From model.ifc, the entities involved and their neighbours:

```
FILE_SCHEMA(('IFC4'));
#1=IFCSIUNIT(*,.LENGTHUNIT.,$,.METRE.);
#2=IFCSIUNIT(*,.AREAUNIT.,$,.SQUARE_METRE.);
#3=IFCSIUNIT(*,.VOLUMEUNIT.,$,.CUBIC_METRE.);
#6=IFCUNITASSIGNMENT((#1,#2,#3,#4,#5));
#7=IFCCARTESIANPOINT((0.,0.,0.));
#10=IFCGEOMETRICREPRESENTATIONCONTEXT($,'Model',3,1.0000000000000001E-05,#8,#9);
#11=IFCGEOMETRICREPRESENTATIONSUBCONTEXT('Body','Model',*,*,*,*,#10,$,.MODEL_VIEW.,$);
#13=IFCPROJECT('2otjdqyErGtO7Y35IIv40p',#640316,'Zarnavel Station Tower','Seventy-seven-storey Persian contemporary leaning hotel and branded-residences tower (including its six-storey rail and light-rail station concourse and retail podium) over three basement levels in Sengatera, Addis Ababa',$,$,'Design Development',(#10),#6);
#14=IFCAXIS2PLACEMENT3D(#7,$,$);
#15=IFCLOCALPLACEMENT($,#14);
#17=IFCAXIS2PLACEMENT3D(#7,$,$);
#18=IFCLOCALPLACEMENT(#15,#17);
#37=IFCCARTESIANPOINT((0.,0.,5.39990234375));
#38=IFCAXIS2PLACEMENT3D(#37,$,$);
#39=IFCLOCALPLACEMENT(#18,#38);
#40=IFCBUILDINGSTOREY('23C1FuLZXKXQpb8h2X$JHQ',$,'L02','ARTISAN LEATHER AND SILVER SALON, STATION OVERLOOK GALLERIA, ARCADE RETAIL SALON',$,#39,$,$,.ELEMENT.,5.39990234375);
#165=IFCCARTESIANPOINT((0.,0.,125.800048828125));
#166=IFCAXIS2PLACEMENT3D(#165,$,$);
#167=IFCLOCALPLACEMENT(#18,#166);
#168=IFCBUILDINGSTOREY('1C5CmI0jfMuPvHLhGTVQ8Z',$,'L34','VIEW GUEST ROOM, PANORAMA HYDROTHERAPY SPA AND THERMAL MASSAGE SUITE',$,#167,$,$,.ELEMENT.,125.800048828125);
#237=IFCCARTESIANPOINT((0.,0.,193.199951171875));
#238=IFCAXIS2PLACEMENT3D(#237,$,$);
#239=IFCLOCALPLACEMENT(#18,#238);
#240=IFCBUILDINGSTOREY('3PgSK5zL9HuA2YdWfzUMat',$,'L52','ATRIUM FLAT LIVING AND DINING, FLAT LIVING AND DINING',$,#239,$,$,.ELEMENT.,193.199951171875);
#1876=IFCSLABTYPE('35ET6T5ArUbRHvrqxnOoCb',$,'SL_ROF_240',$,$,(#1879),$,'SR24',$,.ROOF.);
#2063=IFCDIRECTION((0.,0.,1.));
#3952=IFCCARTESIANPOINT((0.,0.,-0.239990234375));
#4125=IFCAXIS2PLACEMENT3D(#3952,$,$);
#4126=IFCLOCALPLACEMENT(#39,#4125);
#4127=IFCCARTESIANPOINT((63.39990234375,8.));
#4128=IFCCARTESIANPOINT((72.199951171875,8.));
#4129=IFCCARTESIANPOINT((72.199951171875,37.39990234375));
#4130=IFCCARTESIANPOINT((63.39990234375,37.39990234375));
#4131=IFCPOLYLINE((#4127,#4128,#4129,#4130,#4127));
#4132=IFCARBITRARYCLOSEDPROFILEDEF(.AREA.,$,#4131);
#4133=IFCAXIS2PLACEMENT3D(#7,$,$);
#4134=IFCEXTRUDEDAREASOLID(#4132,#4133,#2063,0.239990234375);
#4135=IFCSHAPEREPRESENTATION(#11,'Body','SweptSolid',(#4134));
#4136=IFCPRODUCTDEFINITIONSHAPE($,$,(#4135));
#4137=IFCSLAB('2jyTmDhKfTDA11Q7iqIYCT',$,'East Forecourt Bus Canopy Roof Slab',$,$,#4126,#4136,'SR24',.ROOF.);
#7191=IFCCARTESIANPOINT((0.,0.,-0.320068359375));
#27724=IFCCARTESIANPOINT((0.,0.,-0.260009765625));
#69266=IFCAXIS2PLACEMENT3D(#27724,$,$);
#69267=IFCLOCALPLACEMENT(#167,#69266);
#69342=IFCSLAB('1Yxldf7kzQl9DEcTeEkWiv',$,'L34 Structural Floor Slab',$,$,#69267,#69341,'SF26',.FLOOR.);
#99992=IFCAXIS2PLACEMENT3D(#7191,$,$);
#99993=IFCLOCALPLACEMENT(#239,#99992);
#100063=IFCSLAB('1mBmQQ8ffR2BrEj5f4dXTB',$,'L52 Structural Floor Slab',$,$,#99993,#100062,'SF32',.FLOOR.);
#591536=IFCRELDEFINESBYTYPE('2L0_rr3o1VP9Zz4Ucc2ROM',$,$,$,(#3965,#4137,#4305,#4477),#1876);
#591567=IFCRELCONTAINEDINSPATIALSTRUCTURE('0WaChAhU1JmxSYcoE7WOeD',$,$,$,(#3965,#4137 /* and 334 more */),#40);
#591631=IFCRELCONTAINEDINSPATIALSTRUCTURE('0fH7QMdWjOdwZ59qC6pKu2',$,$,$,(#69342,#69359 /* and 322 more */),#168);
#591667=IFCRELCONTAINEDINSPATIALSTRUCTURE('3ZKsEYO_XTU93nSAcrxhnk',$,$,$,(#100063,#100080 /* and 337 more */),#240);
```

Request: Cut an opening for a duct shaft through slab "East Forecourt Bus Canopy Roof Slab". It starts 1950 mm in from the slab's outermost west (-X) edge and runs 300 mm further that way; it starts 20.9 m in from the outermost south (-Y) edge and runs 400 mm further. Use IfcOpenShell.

```python
import numpy as np
import ifcopenshell
import ifcopenshell.api.feature
import ifcopenshell.api.geometry
import ifcopenshell.api.root
import ifcopenshell.geom
import ifcopenshell.util.placement
import ifcopenshell.util.representation
import ifcopenshell.util.shape
import ifcopenshell.util.unit

model = ifcopenshell.open("model.ifc")
unit_scale = ifcopenshell.util.unit.calculate_unit_scale(model)
settings = ifcopenshell.geom.settings()


def volume(element):
    """Net volume in cubic metres, openings subtracted."""
    shape = ifcopenshell.geom.create_shape(settings, element)
    return ifcopenshell.util.shape.get_volume(shape.geometry)


slab = model.by_id(4137)
before = volume(slab)

# Extent in the slab's own axes, in metres. The edges named are its -X and -Y sides.
slab_shape = ifcopenshell.geom.create_shape(settings, slab)
vertices = ifcopenshell.util.shape.get_vertices(slab_shape.geometry)
x_min, y_min, bottom = vertices.min(axis=0)
top = vertices[:, 2].max()

opening = ifcopenshell.api.root.create_entity(model, ifc_class="IfcOpeningElement", name="Duct shaft opening", predefined_type="OPENING")
context = ifcopenshell.util.representation.get_context(model, "Model", "Body", "MODEL_VIEW")
width, depth = 0.3, 0.4
outline = [(0.0, 0.0), (width, 0.0), (width, depth), (0.0, depth), (0.0, 0.0)]
# Overshoot both faces by 50 mm so the cut is clean.
shape = ifcopenshell.api.geometry.add_slab_representation(
    model, context=context, depth=top - bottom + 0.1, polyline=outline
)
ifcopenshell.api.geometry.assign_representation(model, product=opening, representation=shape)

matrix = ifcopenshell.util.placement.get_local_placement(slab.ObjectPlacement)
matrix[:, 3] = matrix @ np.append(np.array([x_min + 1.95, y_min + 20.9, bottom - 0.05]) / unit_scale, 1.0)
ifcopenshell.api.geometry.edit_object_placement(model, product=opening, matrix=matrix, is_si=False)
ifcopenshell.api.feature.add_feature(model, feature=opening, element=slab)

after = volume(slab)

print(f"slab volume {before:.3f} -> {after:.3f} m3")

model.write("model-out.ifc")
```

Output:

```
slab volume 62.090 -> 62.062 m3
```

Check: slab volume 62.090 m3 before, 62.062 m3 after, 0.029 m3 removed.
